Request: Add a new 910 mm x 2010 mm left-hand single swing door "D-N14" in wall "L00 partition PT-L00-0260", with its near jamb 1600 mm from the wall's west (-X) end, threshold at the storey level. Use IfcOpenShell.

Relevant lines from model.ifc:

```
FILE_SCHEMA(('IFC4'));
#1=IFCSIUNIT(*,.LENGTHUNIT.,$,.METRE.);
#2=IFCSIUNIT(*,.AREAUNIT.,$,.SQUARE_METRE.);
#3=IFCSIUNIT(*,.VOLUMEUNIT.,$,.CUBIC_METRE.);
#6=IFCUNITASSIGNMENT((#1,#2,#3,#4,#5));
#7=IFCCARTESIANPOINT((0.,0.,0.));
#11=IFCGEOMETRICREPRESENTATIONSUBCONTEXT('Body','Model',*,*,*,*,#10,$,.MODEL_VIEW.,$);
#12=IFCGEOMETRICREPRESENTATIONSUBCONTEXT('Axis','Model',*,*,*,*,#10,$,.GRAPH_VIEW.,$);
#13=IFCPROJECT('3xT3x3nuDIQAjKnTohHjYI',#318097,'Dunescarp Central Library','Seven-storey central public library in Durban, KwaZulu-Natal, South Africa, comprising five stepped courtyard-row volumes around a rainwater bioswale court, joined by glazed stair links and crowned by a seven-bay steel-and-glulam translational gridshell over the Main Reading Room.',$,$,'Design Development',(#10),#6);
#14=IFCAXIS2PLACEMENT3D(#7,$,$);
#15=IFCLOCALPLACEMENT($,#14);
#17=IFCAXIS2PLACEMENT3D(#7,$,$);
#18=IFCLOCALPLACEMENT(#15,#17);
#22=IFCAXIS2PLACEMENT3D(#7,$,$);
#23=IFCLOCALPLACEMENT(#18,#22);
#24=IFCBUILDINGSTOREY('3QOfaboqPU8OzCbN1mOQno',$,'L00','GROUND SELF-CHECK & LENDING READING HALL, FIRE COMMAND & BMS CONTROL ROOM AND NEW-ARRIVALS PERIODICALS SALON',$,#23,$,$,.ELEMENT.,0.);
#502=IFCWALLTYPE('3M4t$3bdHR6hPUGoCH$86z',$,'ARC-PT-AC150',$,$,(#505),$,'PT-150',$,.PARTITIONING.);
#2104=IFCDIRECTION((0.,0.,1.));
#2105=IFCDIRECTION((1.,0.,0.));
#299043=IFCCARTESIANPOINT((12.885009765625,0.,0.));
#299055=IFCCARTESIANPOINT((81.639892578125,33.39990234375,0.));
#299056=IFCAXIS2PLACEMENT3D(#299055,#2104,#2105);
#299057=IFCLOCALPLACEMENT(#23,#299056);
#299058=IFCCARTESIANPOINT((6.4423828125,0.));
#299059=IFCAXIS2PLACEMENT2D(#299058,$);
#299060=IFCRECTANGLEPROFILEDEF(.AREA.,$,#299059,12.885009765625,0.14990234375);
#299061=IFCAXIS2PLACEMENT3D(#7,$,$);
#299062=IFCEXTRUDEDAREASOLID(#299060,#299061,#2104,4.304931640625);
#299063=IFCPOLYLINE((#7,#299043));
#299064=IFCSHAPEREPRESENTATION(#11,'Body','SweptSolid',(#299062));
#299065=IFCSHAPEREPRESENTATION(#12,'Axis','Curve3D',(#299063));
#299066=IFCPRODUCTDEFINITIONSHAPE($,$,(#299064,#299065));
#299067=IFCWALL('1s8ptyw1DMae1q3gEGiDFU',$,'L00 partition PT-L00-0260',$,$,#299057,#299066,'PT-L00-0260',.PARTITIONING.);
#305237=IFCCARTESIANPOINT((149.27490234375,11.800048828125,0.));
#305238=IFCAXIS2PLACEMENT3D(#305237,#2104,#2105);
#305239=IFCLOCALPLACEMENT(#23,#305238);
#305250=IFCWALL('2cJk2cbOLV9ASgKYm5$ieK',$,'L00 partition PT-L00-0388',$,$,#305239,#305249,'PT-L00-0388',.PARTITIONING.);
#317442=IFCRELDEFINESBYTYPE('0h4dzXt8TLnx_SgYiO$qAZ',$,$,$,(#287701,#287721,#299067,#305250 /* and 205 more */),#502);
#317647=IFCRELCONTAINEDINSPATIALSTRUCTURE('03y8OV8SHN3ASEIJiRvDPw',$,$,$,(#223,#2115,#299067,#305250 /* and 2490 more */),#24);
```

```python
import numpy as np
import ifcopenshell
import ifcopenshell.api.feature
import ifcopenshell.api.geometry
import ifcopenshell.api.root
import ifcopenshell.api.spatial
import ifcopenshell.geom
import ifcopenshell.util.element
import ifcopenshell.util.placement
import ifcopenshell.util.representation
import ifcopenshell.util.shape
import ifcopenshell.util.unit

model = ifcopenshell.open("model.ifc")
unit_scale = ifcopenshell.util.unit.calculate_unit_scale(model)
settings = ifcopenshell.geom.settings()


def volume(element):
    """Net volume in cubic metres, openings subtracted."""
    shape = ifcopenshell.geom.create_shape(settings, element)
    return ifcopenshell.util.shape.get_volume(shape.geometry)


wall = model.by_id(299067)
storey = ifcopenshell.util.element.get_container(wall, ifc_class="IfcBuildingStorey")
context = ifcopenshell.util.representation.get_context(model, "Model", "Body", "MODEL_VIEW")
before = volume(wall)

width, height, from_end, sill = 0.91, 2.01, 1.6, 0.0  # metres

# The wall runs along its own X axis, and the end named is its -X end.
wall_shape = ifcopenshell.geom.create_shape(settings, wall)
x, y, z = ifcopenshell.util.shape.get_vertices(wall_shape.geometry).T
start = x.min() + from_end
face, thickness = float(y.min()), float(y.max() - y.min())
wall_matrix = ifcopenshell.util.placement.get_local_placement(wall.ObjectPlacement)
level = ifcopenshell.util.placement.get_local_placement(storey.ObjectPlacement)[2, 3]


def in_wall(x, y):
    """Placement at x, y metres in the wall's axes, at sill height."""
    matrix = wall_matrix.copy()
    matrix[:, 3] = wall_matrix @ np.array([x / unit_scale, y / unit_scale, 0.0, 1.0])
    matrix[2, 3] = level + sill / unit_scale
    return matrix


# Opening: a box that overshoots both wall faces by 50 mm.
opening = ifcopenshell.api.root.create_entity(model, ifc_class="IfcOpeningElement", predefined_type="OPENING")
box = ifcopenshell.api.geometry.add_wall_representation(
    model, context=context, length=width, height=height, thickness=thickness + 0.1
)
ifcopenshell.api.geometry.assign_representation(model, product=opening, representation=box)
ifcopenshell.api.geometry.edit_object_placement(model, product=opening, matrix=in_wall(start, face - 0.05), is_si=False)
ifcopenshell.api.feature.add_feature(model, feature=opening, element=wall)

door = ifcopenshell.api.root.create_entity(model, ifc_class="IfcDoor", name="D-N14", predefined_type="DOOR")
door.OverallWidth, door.OverallHeight = width / unit_scale, height / unit_scale
door.OperationType = "SINGLE_SWING_LEFT"
body = ifcopenshell.api.geometry.add_door_representation(
    model,
    context=context,
    overall_width=door.OverallWidth,
    overall_height=door.OverallHeight,
    operation_type="SINGLE_SWING_LEFT",
    lining_properties={"LiningDepth": thickness / unit_scale, "ThresholdDepth": thickness / unit_scale},
)
ifcopenshell.api.geometry.assign_representation(model, product=door, representation=body)
ifcopenshell.api.spatial.assign_container(model, products=[door], relating_structure=storey)
ifcopenshell.api.feature.add_filling(model, opening=opening, element=door)

# The lining spans the wall, so the door starts at the wall face.
ifcopenshell.api.geometry.edit_object_placement(model, product=door, matrix=in_wall(start, face), is_si=False)

after = volume(wall)

print(f"wall volume {before:.3f} -> {after:.3f} m3")

model.write("model-out.ifc")
```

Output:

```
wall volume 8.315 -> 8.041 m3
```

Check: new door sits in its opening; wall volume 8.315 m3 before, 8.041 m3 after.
